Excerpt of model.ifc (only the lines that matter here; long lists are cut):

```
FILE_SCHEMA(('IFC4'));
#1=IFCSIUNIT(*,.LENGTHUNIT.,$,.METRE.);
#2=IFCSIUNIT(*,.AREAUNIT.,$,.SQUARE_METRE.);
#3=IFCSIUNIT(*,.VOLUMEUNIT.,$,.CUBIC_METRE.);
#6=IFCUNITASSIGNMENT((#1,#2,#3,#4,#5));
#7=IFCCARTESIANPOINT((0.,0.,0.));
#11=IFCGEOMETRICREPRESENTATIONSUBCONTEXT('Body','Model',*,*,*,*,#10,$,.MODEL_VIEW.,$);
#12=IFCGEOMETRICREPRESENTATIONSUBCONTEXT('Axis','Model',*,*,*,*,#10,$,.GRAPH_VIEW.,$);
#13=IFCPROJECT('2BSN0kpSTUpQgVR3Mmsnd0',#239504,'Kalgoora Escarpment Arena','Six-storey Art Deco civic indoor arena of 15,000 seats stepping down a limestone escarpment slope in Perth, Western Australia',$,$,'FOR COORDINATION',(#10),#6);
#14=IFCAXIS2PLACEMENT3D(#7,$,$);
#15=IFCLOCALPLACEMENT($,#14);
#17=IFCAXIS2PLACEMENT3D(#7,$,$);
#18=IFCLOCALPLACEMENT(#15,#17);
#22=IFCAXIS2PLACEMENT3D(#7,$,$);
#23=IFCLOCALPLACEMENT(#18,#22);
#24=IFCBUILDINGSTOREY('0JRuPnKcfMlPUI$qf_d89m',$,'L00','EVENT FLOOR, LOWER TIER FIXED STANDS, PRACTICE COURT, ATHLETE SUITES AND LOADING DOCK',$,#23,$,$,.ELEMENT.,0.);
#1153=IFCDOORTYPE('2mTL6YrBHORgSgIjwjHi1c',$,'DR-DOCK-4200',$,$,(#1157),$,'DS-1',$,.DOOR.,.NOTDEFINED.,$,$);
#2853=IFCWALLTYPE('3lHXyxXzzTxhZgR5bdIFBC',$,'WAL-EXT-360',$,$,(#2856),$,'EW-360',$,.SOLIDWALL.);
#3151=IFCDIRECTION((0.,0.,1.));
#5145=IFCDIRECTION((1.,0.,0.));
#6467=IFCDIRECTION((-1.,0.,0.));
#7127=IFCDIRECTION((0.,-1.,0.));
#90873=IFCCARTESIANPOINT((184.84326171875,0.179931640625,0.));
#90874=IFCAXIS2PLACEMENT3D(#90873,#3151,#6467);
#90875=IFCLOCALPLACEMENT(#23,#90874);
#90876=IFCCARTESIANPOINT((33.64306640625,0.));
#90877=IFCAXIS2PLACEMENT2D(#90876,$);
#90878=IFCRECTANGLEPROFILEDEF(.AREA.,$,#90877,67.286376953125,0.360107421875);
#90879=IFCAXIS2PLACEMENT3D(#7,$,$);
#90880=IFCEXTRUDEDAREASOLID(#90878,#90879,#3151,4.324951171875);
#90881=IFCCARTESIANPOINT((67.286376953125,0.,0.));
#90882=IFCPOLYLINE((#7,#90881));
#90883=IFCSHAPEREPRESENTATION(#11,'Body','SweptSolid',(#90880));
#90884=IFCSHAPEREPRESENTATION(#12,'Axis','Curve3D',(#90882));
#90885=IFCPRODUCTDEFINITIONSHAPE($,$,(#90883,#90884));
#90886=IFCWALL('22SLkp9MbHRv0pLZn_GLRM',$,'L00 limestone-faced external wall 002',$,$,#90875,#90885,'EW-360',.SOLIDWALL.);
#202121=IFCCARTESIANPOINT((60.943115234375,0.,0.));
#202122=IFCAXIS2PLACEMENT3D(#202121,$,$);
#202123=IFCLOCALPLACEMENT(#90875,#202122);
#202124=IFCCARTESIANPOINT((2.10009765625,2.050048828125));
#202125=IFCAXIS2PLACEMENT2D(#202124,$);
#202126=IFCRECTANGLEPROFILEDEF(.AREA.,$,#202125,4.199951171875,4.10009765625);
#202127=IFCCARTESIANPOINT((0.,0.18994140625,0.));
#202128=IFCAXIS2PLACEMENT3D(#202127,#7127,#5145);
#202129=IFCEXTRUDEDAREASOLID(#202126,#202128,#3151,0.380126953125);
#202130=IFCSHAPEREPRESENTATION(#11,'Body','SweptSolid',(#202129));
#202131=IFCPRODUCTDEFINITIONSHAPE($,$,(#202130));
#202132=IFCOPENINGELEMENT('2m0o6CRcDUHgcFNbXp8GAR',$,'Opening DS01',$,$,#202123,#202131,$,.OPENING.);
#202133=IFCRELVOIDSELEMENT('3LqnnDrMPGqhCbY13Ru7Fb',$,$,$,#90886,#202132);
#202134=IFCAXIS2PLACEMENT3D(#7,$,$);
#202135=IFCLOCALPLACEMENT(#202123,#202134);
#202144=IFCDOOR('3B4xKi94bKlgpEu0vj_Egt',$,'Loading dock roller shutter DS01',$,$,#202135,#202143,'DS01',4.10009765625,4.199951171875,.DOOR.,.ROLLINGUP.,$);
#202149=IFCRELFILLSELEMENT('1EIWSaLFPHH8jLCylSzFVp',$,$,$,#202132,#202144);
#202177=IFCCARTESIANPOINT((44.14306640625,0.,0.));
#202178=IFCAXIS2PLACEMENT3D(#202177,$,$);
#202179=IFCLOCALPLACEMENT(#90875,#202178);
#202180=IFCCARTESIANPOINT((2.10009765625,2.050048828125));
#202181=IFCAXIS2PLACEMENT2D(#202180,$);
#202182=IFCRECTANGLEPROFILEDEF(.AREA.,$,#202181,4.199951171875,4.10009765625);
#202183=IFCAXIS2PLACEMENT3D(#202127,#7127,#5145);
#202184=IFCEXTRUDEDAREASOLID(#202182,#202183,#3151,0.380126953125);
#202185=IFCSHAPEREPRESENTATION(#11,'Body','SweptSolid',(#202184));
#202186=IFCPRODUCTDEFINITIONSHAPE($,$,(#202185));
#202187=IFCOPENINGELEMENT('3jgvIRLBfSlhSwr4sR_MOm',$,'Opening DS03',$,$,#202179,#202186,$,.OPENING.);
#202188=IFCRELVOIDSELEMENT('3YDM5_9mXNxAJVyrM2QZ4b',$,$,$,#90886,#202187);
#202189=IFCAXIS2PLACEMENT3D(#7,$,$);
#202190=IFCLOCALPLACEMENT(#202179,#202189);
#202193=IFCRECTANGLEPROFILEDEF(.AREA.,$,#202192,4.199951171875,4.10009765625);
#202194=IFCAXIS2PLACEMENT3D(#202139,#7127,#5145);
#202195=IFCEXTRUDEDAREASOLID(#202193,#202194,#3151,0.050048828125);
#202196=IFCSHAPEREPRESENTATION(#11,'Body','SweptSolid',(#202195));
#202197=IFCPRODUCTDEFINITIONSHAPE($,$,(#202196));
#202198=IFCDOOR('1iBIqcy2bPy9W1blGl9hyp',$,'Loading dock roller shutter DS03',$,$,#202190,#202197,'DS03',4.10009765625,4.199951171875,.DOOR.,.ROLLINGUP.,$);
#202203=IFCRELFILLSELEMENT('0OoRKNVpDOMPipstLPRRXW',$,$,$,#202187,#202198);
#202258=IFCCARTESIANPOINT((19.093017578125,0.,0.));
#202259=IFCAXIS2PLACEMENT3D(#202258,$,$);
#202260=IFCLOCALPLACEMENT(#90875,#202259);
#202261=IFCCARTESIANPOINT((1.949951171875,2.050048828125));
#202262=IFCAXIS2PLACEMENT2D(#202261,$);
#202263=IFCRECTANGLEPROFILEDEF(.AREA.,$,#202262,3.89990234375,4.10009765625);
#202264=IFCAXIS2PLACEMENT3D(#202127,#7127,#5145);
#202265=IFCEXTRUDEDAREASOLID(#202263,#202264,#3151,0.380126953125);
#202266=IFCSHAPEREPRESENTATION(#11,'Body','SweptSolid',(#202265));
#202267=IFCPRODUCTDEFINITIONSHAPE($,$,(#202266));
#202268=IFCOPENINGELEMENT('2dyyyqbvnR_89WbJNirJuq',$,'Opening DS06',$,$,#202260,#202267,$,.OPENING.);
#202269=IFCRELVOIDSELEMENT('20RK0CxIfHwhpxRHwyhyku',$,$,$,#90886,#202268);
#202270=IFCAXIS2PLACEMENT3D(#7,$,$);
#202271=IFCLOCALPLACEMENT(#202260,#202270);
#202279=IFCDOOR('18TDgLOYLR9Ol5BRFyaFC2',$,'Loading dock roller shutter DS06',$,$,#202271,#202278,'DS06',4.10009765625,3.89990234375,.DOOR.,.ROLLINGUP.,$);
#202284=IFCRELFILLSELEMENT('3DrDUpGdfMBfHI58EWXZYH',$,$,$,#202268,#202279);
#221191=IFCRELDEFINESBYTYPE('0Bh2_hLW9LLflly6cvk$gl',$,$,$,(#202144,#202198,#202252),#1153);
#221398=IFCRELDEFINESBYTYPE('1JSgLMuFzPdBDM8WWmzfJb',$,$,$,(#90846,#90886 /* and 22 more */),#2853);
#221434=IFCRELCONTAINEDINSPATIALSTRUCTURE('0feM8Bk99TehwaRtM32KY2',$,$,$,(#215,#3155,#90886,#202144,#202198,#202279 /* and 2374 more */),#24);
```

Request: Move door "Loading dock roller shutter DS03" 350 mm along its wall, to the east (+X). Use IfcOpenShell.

```python
import ifcopenshell
import ifcopenshell.api.geometry
import ifcopenshell.util.placement

model = ifcopenshell.open("model.ifc")

door = model.by_guid("1iBIqcy2bPy9W1blGl9hyp")
opening = door.FillsVoids[0].RelatingOpeningElement
wall = opening.VoidsElements[0].RelatingBuildingElement

wall_matrix = ifcopenshell.util.placement.get_local_placement(wall.ObjectPlacement)
shift = wall_matrix[:3, 0] * -0.35
before = ifcopenshell.util.placement.get_local_placement(door.ObjectPlacement)[:3, 3].copy()

# The door is placed relative to its opening, so it follows when the opening moves.
matrix = ifcopenshell.util.placement.get_local_placement(opening.ObjectPlacement)
matrix[:3, 3] += shift
ifcopenshell.api.geometry.edit_object_placement(
    model, product=opening, matrix=matrix, is_si=False, should_transform_children=True
)

after = ifcopenshell.util.placement.get_local_placement(door.ObjectPlacement)[:3, 3]
print("door moved by", (after - before).round(3) + 0.0)

model.write("model_rev.ifc")
```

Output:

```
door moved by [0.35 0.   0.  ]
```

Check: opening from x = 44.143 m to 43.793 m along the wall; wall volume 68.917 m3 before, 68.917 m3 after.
